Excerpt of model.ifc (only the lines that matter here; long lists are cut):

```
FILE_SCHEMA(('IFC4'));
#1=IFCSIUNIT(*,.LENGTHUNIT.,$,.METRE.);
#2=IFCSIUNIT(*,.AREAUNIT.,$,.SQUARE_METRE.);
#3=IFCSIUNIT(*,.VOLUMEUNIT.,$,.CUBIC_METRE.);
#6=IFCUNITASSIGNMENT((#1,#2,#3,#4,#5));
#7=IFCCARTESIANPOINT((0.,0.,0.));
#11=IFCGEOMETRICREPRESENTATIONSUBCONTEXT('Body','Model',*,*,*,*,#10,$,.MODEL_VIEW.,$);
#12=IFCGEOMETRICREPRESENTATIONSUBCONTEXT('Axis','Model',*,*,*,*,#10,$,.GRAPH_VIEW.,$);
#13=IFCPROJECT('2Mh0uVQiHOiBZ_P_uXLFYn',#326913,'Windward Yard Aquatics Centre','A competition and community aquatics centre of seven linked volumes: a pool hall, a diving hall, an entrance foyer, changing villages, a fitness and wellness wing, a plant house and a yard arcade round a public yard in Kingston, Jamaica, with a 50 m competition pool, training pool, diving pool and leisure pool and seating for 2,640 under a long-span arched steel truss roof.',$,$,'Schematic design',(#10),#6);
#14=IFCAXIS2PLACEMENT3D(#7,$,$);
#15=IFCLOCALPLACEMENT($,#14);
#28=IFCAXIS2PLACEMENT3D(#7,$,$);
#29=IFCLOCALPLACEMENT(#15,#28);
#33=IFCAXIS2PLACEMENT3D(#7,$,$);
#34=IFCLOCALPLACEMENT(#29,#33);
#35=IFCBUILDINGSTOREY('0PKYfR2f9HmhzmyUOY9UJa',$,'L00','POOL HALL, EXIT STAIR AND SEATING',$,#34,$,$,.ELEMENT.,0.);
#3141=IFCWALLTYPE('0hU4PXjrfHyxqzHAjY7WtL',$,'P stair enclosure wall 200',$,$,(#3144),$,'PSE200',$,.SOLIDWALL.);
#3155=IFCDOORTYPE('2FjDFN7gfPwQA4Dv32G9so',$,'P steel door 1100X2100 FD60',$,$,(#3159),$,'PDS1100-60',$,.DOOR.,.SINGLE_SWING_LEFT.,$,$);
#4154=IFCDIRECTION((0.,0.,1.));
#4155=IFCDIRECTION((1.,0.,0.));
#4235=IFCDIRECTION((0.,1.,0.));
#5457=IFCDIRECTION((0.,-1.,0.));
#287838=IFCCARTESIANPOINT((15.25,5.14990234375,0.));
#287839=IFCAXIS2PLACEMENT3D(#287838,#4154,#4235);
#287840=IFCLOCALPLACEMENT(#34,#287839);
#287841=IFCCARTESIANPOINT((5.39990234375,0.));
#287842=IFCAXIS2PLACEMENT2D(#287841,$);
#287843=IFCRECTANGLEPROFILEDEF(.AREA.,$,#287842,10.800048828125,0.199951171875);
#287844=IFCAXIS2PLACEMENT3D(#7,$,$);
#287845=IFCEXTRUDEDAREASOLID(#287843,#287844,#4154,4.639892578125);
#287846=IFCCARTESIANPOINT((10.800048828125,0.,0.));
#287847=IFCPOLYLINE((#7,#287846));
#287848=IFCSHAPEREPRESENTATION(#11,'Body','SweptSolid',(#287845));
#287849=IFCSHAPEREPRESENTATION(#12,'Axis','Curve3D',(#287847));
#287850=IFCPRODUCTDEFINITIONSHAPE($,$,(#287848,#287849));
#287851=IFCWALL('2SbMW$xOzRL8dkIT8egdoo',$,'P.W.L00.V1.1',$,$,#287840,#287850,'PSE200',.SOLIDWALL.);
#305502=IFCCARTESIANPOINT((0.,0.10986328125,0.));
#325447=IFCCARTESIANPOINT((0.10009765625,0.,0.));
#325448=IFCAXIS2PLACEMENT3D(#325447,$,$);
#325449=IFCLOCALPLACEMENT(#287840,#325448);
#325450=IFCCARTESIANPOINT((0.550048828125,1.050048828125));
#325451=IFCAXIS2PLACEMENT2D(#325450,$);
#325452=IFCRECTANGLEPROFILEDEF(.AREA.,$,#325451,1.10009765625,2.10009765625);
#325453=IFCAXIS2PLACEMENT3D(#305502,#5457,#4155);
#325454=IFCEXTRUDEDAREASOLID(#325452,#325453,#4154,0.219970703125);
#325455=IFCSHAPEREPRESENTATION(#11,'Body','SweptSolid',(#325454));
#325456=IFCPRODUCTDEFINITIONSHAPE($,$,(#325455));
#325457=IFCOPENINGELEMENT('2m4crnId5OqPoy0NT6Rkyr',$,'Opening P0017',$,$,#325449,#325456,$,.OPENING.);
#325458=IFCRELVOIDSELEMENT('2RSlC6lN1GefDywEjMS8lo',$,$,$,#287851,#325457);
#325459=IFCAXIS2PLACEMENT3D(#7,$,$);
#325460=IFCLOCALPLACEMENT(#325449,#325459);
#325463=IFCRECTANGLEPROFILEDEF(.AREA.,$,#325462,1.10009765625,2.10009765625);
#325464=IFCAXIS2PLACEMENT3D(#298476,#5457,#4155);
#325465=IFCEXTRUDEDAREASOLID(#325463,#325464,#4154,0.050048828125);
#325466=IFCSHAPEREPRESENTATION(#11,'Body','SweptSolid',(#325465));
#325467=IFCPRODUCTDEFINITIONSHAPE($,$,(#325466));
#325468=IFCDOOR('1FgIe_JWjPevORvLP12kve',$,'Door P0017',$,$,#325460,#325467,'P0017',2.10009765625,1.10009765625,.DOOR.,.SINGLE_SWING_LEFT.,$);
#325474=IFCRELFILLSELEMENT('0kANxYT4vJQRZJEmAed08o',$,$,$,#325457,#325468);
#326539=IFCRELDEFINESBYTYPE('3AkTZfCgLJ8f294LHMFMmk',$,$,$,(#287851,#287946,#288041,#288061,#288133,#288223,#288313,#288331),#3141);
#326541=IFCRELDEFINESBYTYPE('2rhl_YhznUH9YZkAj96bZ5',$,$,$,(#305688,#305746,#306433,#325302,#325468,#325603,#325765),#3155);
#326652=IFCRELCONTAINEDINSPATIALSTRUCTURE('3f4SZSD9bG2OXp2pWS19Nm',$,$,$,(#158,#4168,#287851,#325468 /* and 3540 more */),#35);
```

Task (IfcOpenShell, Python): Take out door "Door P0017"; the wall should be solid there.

```python
import ifcopenshell
import ifcopenshell.api.feature
import ifcopenshell.api.root
import ifcopenshell.geom
import ifcopenshell.util.shape

model = ifcopenshell.open("model.ifc")
settings = ifcopenshell.geom.settings()


def volume(element):
    """Net volume in cubic metres, openings subtracted."""
    shape = ifcopenshell.geom.create_shape(settings, element)
    return ifcopenshell.util.shape.get_volume(shape.geometry)


door = model.by_guid("1FgIe_JWjPevORvLP12kve")
opening = door.FillsVoids[0].RelatingOpeningElement
wall = opening.VoidsElements[0].RelatingBuildingElement
before = volume(wall)

ifcopenshell.api.root.remove_product(model, product=door)
ifcopenshell.api.feature.remove_feature(model, feature=opening)

after = volume(wall)

print(f"wall volume {before:.3f} -> {after:.3f} m3")

model.write("model_updated.ifc")
```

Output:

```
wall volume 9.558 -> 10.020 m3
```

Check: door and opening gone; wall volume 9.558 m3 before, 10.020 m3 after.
